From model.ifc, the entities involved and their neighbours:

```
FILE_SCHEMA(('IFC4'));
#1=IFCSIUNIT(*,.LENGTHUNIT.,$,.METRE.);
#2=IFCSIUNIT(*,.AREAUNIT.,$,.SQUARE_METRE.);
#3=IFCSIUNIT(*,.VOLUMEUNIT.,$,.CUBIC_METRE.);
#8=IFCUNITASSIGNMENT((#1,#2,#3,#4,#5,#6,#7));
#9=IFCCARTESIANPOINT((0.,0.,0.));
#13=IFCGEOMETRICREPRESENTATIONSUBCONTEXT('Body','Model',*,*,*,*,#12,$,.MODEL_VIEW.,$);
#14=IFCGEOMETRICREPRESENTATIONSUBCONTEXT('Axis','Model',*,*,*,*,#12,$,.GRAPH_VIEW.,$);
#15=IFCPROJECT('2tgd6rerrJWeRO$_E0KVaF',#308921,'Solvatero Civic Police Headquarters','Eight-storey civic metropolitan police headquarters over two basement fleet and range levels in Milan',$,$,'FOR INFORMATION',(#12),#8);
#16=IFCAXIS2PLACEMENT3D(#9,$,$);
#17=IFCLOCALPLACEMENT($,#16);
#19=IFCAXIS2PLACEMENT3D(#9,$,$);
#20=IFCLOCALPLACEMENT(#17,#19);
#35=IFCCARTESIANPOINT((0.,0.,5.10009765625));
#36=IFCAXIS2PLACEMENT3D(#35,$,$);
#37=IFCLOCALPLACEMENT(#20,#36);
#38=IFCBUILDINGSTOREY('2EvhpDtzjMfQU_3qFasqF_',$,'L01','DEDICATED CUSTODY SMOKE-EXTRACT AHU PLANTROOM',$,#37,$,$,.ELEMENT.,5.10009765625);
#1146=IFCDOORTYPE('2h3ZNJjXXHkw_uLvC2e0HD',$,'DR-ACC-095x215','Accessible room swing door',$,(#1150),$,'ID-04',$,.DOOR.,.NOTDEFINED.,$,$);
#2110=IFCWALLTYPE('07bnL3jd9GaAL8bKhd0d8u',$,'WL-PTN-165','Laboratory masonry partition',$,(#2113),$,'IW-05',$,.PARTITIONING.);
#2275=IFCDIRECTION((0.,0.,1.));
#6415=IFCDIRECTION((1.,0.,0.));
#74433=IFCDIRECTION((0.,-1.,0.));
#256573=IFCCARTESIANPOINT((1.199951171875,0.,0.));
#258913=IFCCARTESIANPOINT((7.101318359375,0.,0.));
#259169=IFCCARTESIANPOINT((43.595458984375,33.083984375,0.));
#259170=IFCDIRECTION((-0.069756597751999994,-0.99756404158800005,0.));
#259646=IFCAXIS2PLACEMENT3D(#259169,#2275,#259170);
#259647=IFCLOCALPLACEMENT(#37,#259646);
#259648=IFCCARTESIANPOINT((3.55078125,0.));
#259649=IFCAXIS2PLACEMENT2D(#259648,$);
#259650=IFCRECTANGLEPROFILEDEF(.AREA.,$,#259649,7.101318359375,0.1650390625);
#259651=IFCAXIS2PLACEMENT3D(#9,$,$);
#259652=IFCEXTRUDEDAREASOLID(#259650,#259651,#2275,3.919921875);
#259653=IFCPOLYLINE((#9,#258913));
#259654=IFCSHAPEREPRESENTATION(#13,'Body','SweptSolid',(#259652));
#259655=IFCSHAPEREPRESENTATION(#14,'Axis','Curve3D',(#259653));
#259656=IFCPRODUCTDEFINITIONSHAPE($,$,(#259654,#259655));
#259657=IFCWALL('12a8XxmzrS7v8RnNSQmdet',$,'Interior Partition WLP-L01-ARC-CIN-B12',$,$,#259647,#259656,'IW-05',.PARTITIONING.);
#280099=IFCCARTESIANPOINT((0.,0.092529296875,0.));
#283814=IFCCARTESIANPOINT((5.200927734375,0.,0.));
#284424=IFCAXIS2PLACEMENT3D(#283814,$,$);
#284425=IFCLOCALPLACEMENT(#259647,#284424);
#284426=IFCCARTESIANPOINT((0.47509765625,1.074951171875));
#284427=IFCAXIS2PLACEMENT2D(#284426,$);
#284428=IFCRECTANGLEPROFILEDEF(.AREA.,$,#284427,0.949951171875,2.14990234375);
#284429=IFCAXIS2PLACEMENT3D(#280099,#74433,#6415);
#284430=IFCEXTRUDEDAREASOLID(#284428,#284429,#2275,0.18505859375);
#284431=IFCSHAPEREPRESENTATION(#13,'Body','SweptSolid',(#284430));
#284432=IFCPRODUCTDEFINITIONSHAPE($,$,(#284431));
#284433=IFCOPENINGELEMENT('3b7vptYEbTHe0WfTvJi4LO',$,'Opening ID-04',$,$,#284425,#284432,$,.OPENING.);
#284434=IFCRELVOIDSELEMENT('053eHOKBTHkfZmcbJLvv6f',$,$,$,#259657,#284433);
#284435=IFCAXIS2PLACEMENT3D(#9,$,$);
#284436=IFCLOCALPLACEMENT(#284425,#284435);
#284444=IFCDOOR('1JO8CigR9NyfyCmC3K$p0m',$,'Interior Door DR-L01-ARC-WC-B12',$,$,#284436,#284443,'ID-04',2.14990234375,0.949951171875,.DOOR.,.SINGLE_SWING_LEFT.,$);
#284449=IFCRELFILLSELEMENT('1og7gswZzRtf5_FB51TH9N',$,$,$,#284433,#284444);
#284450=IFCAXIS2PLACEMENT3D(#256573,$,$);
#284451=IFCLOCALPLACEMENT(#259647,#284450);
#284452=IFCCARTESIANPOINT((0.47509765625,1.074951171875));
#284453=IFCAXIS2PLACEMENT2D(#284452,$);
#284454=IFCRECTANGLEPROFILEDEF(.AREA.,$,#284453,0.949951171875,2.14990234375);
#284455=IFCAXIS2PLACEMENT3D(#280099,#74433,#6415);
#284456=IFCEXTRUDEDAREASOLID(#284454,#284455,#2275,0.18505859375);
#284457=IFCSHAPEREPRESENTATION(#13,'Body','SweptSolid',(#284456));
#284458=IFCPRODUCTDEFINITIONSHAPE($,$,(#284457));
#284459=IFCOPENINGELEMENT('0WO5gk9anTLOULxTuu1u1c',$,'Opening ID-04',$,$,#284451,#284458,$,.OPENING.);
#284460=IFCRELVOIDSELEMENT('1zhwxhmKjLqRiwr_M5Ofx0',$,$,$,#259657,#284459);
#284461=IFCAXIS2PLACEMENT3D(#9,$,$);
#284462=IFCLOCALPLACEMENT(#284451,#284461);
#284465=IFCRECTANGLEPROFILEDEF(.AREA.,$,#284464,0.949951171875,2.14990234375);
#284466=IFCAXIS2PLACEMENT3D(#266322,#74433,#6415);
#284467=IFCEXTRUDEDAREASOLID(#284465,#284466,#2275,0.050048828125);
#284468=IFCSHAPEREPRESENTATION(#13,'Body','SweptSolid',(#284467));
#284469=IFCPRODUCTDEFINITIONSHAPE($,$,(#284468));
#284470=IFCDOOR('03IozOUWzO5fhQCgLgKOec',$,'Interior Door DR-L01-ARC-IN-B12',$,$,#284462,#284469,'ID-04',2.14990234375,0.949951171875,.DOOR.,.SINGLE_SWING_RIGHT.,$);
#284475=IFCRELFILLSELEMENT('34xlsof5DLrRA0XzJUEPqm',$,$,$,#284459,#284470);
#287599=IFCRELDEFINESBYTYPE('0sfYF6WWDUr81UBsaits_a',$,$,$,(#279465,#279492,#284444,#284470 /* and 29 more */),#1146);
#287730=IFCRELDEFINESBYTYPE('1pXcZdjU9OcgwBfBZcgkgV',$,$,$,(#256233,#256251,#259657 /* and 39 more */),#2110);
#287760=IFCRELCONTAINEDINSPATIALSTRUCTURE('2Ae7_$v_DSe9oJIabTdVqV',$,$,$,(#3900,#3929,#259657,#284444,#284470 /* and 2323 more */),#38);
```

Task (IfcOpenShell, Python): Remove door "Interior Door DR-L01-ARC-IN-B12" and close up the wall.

```python
import ifcopenshell
import ifcopenshell.api.feature
import ifcopenshell.api.root
import ifcopenshell.geom
import ifcopenshell.util.shape

model = ifcopenshell.open("model.ifc")
settings = ifcopenshell.geom.settings()


def volume(element):
    """Net volume in cubic metres, openings subtracted."""
    shape = ifcopenshell.geom.create_shape(settings, element)
    return ifcopenshell.util.shape.get_volume(shape.geometry)


door = model.by_guid("03IozOUWzO5fhQCgLgKOec")
opening = door.FillsVoids[0].RelatingOpeningElement
wall = opening.VoidsElements[0].RelatingBuildingElement
before = volume(wall)

ifcopenshell.api.root.remove_product(model, product=door)
ifcopenshell.api.feature.remove_feature(model, feature=opening)

after = volume(wall)

print(f"wall volume {before:.3f} -> {after:.3f} m3")

model.write("model_updated.ifc")
```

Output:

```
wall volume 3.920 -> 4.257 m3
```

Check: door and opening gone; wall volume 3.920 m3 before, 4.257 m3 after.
